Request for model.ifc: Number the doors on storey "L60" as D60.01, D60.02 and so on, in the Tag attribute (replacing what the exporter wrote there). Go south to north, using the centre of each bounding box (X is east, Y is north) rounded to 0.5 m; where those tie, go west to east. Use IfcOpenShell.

First a look at what the model holds.

```python
import ifcopenshell
import ifcopenshell.util.element
import ifcopenshell.util.placement

model = ifcopenshell.open("model.ifc")
print(model.schema)
storey = next(s for s in model.by_type("IfcBuildingStorey") if s.Name == "L60")
doors = [e for e in ifcopenshell.util.element.get_decomposition(storey) if e.is_a("IfcDoor")]
for e in sorted(doors, key=lambda e: e.id()):
    origin = ifcopenshell.util.placement.get_local_placement(e.ObjectPlacement)[:3, 3]
    print(e.id(), e.Tag, e.Name, origin.round(2) + 0.0, sep=" | ")
```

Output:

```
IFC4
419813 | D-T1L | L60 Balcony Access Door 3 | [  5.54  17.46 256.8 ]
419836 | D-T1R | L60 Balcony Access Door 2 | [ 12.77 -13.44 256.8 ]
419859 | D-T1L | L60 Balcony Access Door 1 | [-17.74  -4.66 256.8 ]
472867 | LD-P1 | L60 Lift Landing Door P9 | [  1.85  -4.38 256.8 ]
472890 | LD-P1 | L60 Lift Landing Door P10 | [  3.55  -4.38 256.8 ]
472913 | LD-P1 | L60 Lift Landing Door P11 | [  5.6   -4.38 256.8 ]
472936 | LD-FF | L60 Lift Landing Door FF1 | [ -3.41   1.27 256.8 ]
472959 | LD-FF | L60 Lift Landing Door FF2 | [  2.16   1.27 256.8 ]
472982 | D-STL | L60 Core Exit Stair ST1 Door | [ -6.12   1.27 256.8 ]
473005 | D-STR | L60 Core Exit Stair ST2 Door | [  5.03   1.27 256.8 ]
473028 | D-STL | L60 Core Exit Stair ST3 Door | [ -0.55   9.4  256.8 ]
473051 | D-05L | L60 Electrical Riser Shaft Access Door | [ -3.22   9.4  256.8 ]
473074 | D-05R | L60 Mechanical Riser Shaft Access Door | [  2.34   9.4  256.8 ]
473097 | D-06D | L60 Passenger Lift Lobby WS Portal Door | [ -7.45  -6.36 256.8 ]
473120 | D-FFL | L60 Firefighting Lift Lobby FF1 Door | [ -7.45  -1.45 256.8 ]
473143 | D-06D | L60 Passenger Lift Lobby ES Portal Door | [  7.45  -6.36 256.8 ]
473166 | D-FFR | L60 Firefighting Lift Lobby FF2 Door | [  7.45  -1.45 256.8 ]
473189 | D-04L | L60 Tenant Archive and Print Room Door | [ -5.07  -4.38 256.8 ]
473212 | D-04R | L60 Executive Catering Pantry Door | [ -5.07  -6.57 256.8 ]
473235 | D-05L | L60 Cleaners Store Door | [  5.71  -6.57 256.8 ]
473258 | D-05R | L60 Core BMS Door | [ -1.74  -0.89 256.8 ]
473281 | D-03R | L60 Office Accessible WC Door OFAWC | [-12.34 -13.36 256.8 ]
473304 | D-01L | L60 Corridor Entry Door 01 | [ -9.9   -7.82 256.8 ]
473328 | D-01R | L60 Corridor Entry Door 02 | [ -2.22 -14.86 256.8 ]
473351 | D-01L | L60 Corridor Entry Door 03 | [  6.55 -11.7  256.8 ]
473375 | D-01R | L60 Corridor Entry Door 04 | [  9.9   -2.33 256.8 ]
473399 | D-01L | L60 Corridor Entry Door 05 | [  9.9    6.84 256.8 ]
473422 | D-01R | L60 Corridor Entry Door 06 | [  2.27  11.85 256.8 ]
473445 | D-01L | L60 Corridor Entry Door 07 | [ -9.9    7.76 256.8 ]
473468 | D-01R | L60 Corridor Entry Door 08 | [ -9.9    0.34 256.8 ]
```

```python
import ifcopenshell
import ifcopenshell.geom
import ifcopenshell.util.element
import ifcopenshell.util.shape

model = ifcopenshell.open("model.ifc")
settings = ifcopenshell.geom.settings()
settings.set("use-world-coords", True)


def centre(element):
    shape = ifcopenshell.geom.create_shape(settings, element)
    return ifcopenshell.util.shape.get_bbox_centroid(shape.geometry)


storey = next(s for s in model.by_type("IfcBuildingStorey") if s.Name == "L60")
doors = [e for e in ifcopenshell.util.element.get_decomposition(storey) if e.is_a("IfcDoor")]

# Insertion points can sit at a corner or the storey origin, so sort by the geometry (in metres).
centres = {e: centre(e) for e in doors}
doors.sort(key=lambda e: (round(centres[e][1] / 0.5), centres[e][0]))

for i, e in enumerate(doors, start=1):
    number = f"D60.{i:02d}"
    e.Tag = number
    print(e.id(), number)

model.write("model-out.ifc")
```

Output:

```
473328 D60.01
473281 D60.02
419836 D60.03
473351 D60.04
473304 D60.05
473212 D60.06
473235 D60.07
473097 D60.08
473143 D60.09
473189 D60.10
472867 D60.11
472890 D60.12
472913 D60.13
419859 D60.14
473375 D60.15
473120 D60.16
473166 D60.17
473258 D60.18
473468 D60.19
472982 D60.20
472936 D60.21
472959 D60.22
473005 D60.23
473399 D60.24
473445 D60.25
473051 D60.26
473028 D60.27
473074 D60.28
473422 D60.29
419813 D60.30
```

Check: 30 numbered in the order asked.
